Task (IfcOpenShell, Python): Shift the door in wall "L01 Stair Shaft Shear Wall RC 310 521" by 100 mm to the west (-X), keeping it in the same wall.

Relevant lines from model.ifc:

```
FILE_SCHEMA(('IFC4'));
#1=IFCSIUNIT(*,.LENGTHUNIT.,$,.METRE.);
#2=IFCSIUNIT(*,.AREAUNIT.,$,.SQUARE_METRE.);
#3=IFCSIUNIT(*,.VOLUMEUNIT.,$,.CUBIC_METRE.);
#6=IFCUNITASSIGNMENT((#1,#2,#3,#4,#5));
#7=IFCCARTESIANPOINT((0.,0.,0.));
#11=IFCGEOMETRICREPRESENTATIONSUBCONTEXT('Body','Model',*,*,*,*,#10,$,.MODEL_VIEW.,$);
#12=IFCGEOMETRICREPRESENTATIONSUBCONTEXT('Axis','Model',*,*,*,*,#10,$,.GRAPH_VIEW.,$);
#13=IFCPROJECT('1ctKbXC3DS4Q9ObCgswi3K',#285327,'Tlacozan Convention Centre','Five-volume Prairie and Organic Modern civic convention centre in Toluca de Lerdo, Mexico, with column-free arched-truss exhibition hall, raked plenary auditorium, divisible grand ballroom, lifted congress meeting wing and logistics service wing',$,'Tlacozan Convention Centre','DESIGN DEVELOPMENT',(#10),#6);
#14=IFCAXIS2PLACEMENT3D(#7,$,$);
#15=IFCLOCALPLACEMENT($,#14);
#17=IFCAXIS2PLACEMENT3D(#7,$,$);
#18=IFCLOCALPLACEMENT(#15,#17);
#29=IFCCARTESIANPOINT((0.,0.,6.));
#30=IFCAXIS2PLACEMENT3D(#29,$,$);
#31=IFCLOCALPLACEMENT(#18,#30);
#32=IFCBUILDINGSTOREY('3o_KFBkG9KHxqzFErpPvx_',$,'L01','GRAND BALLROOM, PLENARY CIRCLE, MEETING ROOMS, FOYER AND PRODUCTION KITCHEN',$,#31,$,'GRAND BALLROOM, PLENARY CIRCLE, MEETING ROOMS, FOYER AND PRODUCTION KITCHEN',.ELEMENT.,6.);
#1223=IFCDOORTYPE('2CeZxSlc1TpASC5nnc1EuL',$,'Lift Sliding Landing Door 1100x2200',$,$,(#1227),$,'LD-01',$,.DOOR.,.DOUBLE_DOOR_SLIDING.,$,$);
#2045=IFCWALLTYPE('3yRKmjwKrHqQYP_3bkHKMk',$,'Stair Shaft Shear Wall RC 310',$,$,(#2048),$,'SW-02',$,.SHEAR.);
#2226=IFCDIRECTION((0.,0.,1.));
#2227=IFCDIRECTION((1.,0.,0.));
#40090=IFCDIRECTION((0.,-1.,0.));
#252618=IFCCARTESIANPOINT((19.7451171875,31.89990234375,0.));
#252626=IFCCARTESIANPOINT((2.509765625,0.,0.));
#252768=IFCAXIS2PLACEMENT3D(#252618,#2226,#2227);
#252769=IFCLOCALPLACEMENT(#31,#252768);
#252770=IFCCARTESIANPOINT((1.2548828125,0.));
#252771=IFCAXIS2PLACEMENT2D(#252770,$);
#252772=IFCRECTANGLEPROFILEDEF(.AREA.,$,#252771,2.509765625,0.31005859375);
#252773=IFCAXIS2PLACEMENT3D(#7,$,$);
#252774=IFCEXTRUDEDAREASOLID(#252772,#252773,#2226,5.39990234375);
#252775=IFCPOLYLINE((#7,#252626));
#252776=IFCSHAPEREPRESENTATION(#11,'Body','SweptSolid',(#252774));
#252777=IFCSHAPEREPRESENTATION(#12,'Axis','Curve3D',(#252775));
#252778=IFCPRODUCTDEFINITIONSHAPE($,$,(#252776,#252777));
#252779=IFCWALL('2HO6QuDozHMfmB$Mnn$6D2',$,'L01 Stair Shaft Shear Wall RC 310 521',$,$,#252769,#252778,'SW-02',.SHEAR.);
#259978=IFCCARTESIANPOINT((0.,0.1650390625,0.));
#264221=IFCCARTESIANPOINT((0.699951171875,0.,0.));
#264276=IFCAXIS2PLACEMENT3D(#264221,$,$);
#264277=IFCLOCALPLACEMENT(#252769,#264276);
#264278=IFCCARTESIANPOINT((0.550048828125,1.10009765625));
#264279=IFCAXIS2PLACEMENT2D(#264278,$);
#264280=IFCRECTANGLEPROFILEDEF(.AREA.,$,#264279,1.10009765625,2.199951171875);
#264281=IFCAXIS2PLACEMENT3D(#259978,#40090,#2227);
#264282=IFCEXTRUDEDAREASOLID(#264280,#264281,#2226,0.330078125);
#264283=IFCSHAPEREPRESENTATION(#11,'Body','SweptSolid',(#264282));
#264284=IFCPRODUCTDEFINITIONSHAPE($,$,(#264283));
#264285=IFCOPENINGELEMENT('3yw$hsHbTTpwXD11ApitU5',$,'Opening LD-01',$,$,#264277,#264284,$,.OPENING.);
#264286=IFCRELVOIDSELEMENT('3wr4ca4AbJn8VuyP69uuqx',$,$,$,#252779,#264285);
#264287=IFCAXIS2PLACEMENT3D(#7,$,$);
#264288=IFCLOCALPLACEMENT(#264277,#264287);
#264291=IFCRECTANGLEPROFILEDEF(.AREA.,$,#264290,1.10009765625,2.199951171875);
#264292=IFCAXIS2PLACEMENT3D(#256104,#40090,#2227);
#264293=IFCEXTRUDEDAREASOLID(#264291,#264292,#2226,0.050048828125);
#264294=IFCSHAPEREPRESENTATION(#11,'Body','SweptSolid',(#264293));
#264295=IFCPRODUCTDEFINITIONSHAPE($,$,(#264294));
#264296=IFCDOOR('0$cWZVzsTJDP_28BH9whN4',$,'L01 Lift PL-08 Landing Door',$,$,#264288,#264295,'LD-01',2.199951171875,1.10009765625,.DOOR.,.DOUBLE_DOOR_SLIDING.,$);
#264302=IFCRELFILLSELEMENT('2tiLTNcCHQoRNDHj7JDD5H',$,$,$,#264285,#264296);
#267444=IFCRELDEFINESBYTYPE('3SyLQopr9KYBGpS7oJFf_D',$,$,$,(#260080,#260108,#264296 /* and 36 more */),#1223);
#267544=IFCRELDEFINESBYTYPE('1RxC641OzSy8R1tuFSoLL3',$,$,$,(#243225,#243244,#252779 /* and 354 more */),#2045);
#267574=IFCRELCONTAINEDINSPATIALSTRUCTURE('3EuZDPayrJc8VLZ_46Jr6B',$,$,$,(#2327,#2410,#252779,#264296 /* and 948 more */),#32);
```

```python
import ifcopenshell
import ifcopenshell.api.geometry
import ifcopenshell.util.placement

model = ifcopenshell.open("model.ifc")

door = model.by_id(264296)
opening = door.FillsVoids[0].RelatingOpeningElement
wall = opening.VoidsElements[0].RelatingBuildingElement

wall_matrix = ifcopenshell.util.placement.get_local_placement(wall.ObjectPlacement)
shift = wall_matrix[:3, 0] * -0.1
before = ifcopenshell.util.placement.get_local_placement(door.ObjectPlacement)[:3, 3].copy()

# The door is placed relative to its opening, so it follows when the opening moves.
matrix = ifcopenshell.util.placement.get_local_placement(opening.ObjectPlacement)
matrix[:3, 3] += shift
ifcopenshell.api.geometry.edit_object_placement(
    model, product=opening, matrix=matrix, is_si=False, should_transform_children=True
)

after = ifcopenshell.util.placement.get_local_placement(door.ObjectPlacement)[:3, 3]
print("door moved by", (after - before).round(3) + 0.0)

model.write("model_rev.ifc")
```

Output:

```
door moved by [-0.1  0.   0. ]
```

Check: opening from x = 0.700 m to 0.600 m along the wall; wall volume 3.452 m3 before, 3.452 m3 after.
